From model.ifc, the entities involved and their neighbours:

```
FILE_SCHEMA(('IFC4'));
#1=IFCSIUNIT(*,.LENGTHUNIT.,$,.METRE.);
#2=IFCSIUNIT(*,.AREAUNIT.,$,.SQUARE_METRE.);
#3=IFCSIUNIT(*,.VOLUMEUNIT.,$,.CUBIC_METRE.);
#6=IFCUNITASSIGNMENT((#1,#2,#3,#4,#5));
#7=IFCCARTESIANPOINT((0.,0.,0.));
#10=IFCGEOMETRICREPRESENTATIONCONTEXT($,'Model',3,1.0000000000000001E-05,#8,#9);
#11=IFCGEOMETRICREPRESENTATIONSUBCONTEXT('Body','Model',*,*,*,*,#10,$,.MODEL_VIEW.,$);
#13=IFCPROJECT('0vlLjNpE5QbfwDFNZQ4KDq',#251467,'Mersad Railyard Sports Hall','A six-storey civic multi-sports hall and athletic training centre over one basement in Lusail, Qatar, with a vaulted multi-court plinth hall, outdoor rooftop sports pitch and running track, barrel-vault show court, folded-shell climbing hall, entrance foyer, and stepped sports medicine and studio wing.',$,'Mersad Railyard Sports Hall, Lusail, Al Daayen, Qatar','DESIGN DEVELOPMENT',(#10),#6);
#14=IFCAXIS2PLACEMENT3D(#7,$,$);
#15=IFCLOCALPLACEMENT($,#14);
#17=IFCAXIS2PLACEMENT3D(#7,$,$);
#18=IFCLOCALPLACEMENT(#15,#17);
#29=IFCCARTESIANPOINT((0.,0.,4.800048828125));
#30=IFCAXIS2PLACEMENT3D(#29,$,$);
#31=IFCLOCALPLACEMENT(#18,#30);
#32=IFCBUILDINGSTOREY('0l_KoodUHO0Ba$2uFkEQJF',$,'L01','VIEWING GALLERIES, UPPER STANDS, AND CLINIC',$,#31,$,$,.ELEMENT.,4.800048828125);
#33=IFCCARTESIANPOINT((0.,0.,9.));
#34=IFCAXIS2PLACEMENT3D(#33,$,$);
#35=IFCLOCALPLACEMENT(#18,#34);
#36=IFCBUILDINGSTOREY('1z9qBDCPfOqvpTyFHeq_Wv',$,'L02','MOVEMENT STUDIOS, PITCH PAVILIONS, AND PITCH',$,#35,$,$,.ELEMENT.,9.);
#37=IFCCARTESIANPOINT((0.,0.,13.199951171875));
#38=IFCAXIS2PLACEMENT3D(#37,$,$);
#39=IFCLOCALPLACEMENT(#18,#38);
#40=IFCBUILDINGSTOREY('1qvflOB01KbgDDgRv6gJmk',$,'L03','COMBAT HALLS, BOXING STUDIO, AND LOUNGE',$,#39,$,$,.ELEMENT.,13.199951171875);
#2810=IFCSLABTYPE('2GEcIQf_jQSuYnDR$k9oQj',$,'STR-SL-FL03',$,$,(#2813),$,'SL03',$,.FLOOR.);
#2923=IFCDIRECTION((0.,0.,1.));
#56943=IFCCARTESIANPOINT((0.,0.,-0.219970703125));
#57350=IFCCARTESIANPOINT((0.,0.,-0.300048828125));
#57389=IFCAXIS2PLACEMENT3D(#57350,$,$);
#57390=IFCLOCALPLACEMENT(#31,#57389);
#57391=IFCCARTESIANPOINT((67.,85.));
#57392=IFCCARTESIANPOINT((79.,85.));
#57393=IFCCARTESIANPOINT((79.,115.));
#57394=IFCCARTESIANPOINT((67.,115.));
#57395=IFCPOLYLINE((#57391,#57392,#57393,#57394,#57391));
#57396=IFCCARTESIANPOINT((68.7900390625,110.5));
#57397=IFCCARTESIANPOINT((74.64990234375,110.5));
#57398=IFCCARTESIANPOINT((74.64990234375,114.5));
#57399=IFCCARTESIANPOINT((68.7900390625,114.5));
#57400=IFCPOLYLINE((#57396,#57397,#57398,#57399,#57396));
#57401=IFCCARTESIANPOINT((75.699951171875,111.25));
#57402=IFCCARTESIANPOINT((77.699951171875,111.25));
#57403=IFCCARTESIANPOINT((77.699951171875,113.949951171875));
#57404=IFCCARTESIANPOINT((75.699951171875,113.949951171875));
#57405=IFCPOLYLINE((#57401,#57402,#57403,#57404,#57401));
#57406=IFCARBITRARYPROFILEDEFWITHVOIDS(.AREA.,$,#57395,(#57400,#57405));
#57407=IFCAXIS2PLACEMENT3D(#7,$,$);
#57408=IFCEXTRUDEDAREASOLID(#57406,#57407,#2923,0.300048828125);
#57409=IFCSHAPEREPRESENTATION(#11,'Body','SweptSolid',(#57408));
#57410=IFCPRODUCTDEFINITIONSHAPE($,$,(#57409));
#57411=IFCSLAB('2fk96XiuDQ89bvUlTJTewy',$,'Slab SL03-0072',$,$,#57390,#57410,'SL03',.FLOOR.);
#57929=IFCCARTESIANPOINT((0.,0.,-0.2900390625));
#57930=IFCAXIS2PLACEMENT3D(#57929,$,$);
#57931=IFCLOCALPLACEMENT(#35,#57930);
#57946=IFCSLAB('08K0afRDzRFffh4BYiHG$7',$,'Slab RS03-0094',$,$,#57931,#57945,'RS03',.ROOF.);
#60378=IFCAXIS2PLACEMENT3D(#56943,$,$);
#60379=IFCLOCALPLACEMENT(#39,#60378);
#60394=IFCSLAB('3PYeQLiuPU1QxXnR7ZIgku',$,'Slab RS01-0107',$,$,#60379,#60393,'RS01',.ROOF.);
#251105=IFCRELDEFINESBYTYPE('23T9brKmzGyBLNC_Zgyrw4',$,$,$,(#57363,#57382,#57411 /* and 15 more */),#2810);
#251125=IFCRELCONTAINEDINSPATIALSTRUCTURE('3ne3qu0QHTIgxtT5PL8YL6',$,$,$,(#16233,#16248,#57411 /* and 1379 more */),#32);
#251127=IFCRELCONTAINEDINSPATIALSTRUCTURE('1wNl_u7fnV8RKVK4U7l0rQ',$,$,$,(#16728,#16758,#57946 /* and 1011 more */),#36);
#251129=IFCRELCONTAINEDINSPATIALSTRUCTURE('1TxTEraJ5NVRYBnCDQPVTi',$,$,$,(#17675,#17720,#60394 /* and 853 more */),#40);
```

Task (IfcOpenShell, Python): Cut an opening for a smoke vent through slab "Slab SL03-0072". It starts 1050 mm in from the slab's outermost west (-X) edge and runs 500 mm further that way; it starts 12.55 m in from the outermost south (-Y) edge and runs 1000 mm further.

```python
import numpy as np
import ifcopenshell
import ifcopenshell.api.feature
import ifcopenshell.api.geometry
import ifcopenshell.api.root
import ifcopenshell.geom
import ifcopenshell.util.placement
import ifcopenshell.util.representation
import ifcopenshell.util.shape
import ifcopenshell.util.unit

model = ifcopenshell.open("model.ifc")
unit_scale = ifcopenshell.util.unit.calculate_unit_scale(model)
settings = ifcopenshell.geom.settings()


def volume(element):
    """Net volume in cubic metres, openings subtracted."""
    shape = ifcopenshell.geom.create_shape(settings, element)
    return ifcopenshell.util.shape.get_volume(shape.geometry)


slab = model.by_guid("2fk96XiuDQ89bvUlTJTewy")
before = volume(slab)

# Extent in the slab's own axes, in metres. The edges named are its -X and -Y sides.
slab_shape = ifcopenshell.geom.create_shape(settings, slab)
vertices = ifcopenshell.util.shape.get_vertices(slab_shape.geometry)
x_min, y_min, bottom = vertices.min(axis=0)
top = vertices[:, 2].max()

opening = ifcopenshell.api.root.create_entity(model, ifc_class="IfcOpeningElement", name="Smoke vent opening", predefined_type="OPENING")
context = ifcopenshell.util.representation.get_context(model, "Model", "Body", "MODEL_VIEW")
width, depth = 0.5, 1
outline = [(0.0, 0.0), (width, 0.0), (width, depth), (0.0, depth), (0.0, 0.0)]
# Overshoot both faces by 50 mm so the cut is clean.
shape = ifcopenshell.api.geometry.add_slab_representation(
    model, context=context, depth=top - bottom + 0.1, polyline=outline
)
ifcopenshell.api.geometry.assign_representation(model, product=opening, representation=shape)

matrix = ifcopenshell.util.placement.get_local_placement(slab.ObjectPlacement)
matrix[:, 3] = matrix @ np.append(np.array([x_min + 1.05, y_min + 12.55, bottom - 0.05]) / unit_scale, 1.0)
ifcopenshell.api.geometry.edit_object_placement(model, product=opening, matrix=matrix, is_si=False)
ifcopenshell.api.feature.add_feature(model, feature=opening, element=slab)

after = volume(slab)

print(f"slab volume {before:.3f} -> {after:.3f} m3")

model.write("model-out.ifc")
```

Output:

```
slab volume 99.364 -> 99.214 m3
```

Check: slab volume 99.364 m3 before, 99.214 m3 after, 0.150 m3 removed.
